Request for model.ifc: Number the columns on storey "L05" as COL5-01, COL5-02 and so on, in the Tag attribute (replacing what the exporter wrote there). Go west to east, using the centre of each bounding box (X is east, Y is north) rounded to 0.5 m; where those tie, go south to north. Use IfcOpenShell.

First a look at what the model holds.

```python
import ifcopenshell
import ifcopenshell.util.element
import ifcopenshell.util.placement

model = ifcopenshell.open("model.ifc")
print(model.schema)
storey = next(s for s in model.by_type("IfcBuildingStorey") if s.Name == "L05")
columns = [e for e in ifcopenshell.util.element.get_decomposition(storey) if e.is_a("IfcColumn")]
for e in sorted(columns, key=lambda e: e.id()):
    origin = ifcopenshell.util.placement.get_local_placement(e.ObjectPlacement)[:3, 3]
    print(e.id(), e.Tag, e.Name, origin.round(2) + 0.0, sep=" | ")
```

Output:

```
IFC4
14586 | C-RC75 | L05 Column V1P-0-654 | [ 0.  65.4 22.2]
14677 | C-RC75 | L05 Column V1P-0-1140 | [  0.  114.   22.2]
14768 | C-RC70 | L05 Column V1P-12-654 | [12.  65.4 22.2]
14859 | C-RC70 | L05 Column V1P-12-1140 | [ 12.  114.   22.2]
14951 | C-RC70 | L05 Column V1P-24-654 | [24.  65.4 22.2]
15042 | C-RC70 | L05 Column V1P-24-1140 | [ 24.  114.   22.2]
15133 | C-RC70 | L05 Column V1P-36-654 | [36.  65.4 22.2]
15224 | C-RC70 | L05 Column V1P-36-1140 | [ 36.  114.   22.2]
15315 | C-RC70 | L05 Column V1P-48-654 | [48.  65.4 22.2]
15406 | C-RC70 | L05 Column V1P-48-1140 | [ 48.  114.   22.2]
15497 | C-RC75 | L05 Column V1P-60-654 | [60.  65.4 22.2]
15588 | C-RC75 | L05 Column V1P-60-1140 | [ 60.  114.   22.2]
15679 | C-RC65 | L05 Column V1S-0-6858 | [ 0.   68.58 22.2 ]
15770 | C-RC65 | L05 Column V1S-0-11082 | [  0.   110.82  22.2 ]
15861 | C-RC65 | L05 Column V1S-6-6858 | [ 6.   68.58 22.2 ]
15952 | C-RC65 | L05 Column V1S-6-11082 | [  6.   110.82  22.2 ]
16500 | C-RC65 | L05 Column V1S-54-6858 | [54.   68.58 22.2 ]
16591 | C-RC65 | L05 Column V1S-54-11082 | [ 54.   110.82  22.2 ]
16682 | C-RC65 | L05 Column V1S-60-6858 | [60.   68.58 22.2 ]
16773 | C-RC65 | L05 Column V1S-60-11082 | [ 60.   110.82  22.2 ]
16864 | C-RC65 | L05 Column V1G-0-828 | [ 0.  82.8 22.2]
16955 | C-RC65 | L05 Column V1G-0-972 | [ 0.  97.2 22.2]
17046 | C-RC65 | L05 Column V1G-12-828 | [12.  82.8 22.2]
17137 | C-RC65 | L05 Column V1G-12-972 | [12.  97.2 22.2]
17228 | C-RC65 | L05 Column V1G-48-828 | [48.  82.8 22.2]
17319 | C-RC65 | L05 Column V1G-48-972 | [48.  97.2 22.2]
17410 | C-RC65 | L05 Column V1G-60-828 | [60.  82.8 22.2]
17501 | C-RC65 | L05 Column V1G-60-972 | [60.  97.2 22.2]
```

```python
import ifcopenshell
import ifcopenshell.geom
import ifcopenshell.util.element
import ifcopenshell.util.shape

model = ifcopenshell.open("model.ifc")
settings = ifcopenshell.geom.settings()
settings.set("use-world-coords", True)


def centre(element):
    shape = ifcopenshell.geom.create_shape(settings, element)
    return ifcopenshell.util.shape.get_bbox_centroid(shape.geometry)


storey = next(s for s in model.by_type("IfcBuildingStorey") if s.Name == "L05")
columns = [e for e in ifcopenshell.util.element.get_decomposition(storey) if e.is_a("IfcColumn")]

# Insertion points can sit at a corner or the storey origin, so sort by the geometry (in metres).
centres = {e: centre(e) for e in columns}
columns.sort(key=lambda e: (round(centres[e][0] / 0.5), centres[e][1]))

for i, e in enumerate(columns, start=1):
    number = f"COL5-{i:02d}"
    e.Tag = number
    print(e.id(), number)

model.write("model_edited.ifc")
```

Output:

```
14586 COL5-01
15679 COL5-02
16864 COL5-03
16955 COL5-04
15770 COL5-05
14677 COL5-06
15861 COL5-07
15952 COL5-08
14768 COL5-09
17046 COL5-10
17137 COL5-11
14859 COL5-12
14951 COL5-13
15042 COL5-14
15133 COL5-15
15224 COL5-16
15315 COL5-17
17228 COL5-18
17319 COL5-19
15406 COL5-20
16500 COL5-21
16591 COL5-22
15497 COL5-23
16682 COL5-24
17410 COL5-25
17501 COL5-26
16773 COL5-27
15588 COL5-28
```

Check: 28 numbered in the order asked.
